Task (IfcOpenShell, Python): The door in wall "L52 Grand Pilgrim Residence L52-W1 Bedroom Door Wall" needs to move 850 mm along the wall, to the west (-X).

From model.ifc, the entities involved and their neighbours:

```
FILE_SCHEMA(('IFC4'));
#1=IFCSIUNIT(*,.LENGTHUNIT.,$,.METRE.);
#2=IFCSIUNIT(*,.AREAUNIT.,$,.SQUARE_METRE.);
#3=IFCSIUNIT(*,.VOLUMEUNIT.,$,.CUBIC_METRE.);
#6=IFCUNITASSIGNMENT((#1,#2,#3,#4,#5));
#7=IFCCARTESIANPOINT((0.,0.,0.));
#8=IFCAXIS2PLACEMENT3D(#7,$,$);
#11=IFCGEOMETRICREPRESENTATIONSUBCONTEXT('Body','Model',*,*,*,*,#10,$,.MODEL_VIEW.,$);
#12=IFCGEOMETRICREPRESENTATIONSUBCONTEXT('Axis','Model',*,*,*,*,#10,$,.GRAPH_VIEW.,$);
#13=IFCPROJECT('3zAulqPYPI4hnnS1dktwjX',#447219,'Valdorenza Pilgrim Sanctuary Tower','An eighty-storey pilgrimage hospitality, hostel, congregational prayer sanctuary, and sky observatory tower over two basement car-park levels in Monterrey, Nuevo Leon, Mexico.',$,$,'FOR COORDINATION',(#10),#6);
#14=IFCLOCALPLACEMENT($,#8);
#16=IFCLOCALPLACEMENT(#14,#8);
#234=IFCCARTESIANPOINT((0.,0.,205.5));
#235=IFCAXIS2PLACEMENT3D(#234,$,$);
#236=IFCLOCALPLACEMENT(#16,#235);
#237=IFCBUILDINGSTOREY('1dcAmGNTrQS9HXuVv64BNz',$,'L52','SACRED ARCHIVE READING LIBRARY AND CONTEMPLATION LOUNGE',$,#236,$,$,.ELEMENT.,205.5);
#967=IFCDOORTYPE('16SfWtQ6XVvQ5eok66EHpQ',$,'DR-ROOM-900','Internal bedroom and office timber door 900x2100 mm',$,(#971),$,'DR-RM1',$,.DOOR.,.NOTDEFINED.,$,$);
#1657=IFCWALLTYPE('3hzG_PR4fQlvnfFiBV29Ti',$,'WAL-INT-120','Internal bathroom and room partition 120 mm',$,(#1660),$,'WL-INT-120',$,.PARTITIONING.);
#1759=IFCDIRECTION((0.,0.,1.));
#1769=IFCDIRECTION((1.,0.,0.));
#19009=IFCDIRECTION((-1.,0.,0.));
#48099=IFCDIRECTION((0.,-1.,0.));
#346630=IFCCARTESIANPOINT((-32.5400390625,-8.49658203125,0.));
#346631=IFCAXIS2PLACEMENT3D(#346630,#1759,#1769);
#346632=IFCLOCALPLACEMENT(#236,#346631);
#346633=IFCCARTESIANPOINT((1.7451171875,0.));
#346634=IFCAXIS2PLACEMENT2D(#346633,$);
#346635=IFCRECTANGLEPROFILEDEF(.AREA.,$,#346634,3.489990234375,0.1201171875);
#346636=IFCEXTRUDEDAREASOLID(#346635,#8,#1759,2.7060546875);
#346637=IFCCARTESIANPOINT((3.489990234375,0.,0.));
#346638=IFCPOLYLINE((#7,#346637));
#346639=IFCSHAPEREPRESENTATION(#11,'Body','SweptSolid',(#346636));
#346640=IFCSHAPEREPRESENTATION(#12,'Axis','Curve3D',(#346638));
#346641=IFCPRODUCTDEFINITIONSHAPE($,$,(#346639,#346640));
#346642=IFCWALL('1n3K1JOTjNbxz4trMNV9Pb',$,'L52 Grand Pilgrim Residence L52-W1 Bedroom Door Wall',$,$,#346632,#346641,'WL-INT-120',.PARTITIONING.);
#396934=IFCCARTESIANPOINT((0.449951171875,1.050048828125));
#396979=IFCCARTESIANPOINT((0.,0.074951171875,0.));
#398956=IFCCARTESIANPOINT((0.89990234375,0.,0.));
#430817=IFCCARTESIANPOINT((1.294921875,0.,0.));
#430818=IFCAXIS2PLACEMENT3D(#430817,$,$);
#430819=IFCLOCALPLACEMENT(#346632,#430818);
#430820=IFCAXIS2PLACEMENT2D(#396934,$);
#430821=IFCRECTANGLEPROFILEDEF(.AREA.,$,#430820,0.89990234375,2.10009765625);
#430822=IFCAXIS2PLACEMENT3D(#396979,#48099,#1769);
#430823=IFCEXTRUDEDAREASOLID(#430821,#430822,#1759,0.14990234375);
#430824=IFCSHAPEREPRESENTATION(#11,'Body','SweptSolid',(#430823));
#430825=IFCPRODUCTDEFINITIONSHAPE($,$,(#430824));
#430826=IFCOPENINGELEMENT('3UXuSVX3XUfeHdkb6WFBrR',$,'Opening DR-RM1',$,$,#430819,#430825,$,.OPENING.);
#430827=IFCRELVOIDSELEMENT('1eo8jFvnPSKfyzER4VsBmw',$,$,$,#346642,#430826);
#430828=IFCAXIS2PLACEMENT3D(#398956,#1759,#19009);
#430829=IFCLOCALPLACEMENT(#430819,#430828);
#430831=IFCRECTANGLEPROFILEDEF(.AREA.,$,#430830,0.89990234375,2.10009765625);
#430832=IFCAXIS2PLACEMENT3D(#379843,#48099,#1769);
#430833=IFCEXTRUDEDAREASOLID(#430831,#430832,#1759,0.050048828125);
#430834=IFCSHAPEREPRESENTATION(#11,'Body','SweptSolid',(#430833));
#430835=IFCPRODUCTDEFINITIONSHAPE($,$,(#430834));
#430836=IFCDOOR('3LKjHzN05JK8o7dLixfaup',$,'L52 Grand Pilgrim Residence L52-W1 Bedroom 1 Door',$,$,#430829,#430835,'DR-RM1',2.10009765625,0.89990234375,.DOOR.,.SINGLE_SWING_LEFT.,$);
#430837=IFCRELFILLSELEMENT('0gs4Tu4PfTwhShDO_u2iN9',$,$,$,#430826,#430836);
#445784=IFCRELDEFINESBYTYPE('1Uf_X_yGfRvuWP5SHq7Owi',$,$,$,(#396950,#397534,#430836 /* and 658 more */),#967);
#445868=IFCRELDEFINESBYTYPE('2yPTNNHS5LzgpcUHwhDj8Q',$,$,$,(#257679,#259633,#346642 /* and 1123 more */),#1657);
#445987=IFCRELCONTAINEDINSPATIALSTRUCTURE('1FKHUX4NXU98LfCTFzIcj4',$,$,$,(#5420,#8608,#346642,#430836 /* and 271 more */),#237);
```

```python
import ifcopenshell
import ifcopenshell.api.geometry
import ifcopenshell.util.placement

model = ifcopenshell.open("model.ifc")

door = model.by_id(430836)
opening = door.FillsVoids[0].RelatingOpeningElement
wall = opening.VoidsElements[0].RelatingBuildingElement

wall_matrix = ifcopenshell.util.placement.get_local_placement(wall.ObjectPlacement)
shift = wall_matrix[:3, 0] * -0.85
before = ifcopenshell.util.placement.get_local_placement(door.ObjectPlacement)[:3, 3].copy()

# The door is placed relative to its opening, so it follows when the opening moves.
matrix = ifcopenshell.util.placement.get_local_placement(opening.ObjectPlacement)
matrix[:3, 3] += shift
ifcopenshell.api.geometry.edit_object_placement(
    model, product=opening, matrix=matrix, is_si=False, should_transform_children=True
)

after = ifcopenshell.util.placement.get_local_placement(door.ObjectPlacement)[:3, 3]
print("door moved by", (after - before).round(3) + 0.0)

model.write("model_edited.ifc")
```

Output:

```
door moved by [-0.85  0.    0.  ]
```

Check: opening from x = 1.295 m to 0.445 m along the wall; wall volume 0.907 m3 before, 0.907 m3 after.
